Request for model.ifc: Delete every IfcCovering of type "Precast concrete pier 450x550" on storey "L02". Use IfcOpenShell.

First a look at what the model holds.

```python
import ifcopenshell
import ifcopenshell.util.element

model = ifcopenshell.open("model.ifc")
print(model.schema)
storey = next(s for s in model.by_type("IfcBuildingStorey") if s.Name == "L02")
coverings = [e for e in ifcopenshell.util.element.get_decomposition(storey) if e.is_a("IfcCovering")]
seen = {}
for e in coverings:
    element_type = ifcopenshell.util.element.get_type(e)
    name = element_type.Name if element_type not in (None, e) else None
    seen[name] = seen.get(name, 0) + 1
for name, count in sorted(seen.items(), key=str):
    print(count, "x", name)
```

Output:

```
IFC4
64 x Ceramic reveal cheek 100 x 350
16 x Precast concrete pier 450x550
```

```python
import ifcopenshell
import ifcopenshell.api.root
import ifcopenshell.util.element

model = ifcopenshell.open("model.ifc")

storey = next(s for s in model.by_type("IfcBuildingStorey") if s.Name == "L02")
coverings = [e for e in ifcopenshell.util.element.get_decomposition(storey) if e.is_a("IfcCovering")]
targets = [e for e in coverings if (t := ifcopenshell.util.element.get_type(e)) not in (None, e) and t.Name == "Precast concrete pier 450x550"]

for e in targets:
    ifcopenshell.api.root.remove_product(model, product=e)
print(len(targets), "removed")

model.write("model-out.ifc")
```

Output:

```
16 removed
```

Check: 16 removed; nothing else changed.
